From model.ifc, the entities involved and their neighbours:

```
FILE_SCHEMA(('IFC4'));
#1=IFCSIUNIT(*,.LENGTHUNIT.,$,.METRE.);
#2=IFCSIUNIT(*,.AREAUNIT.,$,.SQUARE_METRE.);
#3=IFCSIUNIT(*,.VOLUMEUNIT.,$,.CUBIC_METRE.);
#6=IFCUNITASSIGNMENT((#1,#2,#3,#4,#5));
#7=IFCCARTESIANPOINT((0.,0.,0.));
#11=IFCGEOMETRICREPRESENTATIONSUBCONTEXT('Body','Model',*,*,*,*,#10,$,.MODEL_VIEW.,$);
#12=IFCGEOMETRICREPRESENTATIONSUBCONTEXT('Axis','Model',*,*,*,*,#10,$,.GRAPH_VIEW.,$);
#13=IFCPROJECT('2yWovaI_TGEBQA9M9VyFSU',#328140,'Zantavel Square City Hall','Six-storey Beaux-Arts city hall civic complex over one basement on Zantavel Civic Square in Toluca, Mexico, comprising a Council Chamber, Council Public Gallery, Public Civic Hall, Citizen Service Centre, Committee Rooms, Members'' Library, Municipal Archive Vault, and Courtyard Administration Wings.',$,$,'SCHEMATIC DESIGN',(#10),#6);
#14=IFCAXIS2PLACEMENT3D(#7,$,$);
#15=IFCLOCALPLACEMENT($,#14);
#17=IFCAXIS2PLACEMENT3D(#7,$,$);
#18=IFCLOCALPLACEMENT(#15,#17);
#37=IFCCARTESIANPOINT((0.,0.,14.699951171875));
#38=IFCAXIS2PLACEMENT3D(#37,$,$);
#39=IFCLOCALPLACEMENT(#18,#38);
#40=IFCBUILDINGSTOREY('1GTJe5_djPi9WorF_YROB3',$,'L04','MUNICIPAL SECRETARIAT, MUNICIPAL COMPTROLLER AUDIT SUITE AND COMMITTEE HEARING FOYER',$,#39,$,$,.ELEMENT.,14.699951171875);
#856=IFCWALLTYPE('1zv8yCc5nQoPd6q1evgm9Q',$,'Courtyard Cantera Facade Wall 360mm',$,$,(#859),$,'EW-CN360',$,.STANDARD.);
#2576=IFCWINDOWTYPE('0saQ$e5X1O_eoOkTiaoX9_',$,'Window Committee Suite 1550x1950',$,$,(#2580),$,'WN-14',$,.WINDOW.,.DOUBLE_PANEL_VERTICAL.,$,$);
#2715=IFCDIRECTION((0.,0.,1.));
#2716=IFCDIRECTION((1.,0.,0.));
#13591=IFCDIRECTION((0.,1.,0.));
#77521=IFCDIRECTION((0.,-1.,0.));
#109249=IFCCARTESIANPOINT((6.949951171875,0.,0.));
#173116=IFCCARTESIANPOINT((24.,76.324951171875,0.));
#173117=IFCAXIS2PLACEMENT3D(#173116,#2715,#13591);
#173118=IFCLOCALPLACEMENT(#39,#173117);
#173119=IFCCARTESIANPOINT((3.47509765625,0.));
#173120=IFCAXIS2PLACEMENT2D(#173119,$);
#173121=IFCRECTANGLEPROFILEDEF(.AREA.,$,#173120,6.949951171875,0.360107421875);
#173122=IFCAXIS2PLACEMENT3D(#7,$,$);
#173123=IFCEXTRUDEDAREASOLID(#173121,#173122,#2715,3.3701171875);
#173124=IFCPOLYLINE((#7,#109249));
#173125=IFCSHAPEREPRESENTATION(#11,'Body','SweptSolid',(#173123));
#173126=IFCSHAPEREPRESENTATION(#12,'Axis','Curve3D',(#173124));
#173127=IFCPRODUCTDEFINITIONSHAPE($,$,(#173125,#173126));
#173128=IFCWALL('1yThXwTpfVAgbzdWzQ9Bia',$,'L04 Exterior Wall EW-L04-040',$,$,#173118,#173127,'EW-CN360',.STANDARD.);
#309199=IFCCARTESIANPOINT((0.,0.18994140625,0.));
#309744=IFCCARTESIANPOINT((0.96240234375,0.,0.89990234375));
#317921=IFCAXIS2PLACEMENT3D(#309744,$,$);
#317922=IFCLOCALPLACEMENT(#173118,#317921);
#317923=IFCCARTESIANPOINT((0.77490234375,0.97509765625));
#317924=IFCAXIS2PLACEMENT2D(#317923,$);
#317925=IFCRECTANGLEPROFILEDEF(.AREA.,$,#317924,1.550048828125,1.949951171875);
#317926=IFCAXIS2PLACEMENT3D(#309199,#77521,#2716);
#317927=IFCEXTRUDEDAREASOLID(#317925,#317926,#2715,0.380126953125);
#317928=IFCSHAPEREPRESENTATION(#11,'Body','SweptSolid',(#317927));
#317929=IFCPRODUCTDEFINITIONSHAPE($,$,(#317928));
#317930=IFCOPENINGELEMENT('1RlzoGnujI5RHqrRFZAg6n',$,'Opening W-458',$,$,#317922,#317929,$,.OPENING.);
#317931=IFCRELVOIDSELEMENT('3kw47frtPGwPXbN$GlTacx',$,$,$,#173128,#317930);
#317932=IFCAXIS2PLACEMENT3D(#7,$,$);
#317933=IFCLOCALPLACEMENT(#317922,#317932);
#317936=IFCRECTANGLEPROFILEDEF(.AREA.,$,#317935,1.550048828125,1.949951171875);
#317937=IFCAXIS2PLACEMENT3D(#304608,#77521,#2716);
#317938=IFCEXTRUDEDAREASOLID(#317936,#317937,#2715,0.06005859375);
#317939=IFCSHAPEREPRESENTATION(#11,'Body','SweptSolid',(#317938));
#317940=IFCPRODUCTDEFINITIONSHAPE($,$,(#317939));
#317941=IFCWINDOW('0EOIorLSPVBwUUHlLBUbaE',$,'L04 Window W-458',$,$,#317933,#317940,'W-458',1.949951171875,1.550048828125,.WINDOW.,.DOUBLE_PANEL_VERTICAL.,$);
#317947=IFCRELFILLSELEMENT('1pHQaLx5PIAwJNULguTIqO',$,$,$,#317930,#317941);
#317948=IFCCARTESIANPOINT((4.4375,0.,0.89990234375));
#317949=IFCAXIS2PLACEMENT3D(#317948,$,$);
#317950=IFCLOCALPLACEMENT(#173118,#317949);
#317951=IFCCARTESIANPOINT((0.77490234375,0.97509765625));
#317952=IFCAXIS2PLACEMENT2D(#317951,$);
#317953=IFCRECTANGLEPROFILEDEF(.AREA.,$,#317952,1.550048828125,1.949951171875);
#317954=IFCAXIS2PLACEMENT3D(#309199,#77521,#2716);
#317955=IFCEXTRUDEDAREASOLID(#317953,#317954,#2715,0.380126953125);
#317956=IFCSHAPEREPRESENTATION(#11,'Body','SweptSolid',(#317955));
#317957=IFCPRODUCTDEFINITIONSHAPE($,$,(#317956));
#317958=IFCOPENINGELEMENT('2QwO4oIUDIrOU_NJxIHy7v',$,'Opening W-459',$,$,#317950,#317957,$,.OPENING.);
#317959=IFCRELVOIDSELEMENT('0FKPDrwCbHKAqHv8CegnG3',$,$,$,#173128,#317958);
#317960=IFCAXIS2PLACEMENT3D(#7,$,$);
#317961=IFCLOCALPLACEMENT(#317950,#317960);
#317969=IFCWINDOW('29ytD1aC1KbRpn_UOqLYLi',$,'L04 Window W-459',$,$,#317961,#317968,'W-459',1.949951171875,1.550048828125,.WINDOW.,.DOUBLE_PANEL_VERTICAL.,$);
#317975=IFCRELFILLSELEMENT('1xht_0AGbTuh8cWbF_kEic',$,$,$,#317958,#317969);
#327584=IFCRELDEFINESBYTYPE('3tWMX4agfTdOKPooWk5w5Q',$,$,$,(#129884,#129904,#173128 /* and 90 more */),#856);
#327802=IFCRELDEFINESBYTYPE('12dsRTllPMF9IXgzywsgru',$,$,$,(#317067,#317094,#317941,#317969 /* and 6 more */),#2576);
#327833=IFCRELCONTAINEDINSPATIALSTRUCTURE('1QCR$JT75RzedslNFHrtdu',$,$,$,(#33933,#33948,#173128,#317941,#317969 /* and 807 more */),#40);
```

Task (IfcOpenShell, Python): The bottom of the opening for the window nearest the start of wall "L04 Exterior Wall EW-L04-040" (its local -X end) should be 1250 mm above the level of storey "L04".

```python
import numpy as np
import ifcopenshell
import ifcopenshell.api.geometry
import ifcopenshell.geom
import ifcopenshell.util.element
import ifcopenshell.util.placement
import ifcopenshell.util.shape
import ifcopenshell.util.unit

model = ifcopenshell.open("model.ifc")
unit_scale = ifcopenshell.util.unit.calculate_unit_scale(model)

window = model.by_id(317941)
opening = window.FillsVoids[0].RelatingOpeningElement
storey = ifcopenshell.util.element.get_container(window, ifc_class="IfcBuildingStorey")
level = ifcopenshell.util.placement.get_local_placement(storey.ObjectPlacement)[2, 3]

# The opening's origin need not be at the sill, so measure its lowest point.
shape = ifcopenshell.geom.create_shape(ifcopenshell.geom.settings(), opening)
bottom = ifcopenshell.util.shape.get_shape_bottom_elevation(shape, shape.geometry) / unit_scale
dz = level + 1.25 - bottom

shift = np.array([0.0, 0.0, dz])
# The window is placed relative to its opening, so it follows when the opening moves.
matrix = ifcopenshell.util.placement.get_local_placement(opening.ObjectPlacement)
matrix[:3, 3] += shift
ifcopenshell.api.geometry.edit_object_placement(
    model, product=opening, matrix=matrix, is_si=False, should_transform_children=True
)

print(f"moved by {dz * unit_scale:+.3f} m")

model.write("model_edited.ifc")
```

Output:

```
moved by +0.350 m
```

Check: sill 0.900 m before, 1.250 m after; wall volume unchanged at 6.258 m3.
